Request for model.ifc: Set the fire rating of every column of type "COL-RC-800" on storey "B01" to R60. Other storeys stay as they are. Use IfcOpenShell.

First a look at what the model holds.

```python
import ifcopenshell
import ifcopenshell.util.element

model = ifcopenshell.open("model.ifc")
print(model.schema)
storey = next(s for s in model.by_type("IfcBuildingStorey") if s.Name == "B01")
columns = [e for e in ifcopenshell.util.element.get_decomposition(storey) if e.is_a("IfcColumn")]
seen = {}
for e in columns:
    element_type = ifcopenshell.util.element.get_type(e)
    key = (element_type.Name if element_type != e and element_type else None, ifcopenshell.util.element.get_pset(e, "Pset_ColumnCommon", "FireRating"))
    seen[key] = seen.get(key, 0) + 1
for (name, value), count in sorted(seen.items(), key=str):
    print(count, "x", name, "|", value)
```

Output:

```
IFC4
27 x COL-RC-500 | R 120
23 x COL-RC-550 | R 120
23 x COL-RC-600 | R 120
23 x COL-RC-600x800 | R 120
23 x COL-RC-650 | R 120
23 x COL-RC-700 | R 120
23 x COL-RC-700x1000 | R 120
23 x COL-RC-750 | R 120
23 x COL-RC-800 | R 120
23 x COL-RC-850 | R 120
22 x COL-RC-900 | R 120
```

```python
import ifcopenshell
import ifcopenshell.api.pset
import ifcopenshell.util.element

model = ifcopenshell.open("model.ifc")

storey = next(s for s in model.by_type("IfcBuildingStorey") if s.Name == "B01")
columns = [e for e in ifcopenshell.util.element.get_decomposition(storey) if e.is_a("IfcColumn")]

count = 0
for e in columns:
    element_type = ifcopenshell.util.element.get_type(e)
    if element_type in (None, e) or element_type.Name != "COL-RC-800":
        continue
    # add_pset returns the element's existing set when there is one.
    pset = ifcopenshell.api.pset.add_pset(model, product=e, name="Pset_ColumnCommon")
    ifcopenshell.api.pset.edit_pset(model, pset=pset, properties={"FireRating": "R60"})
    count += 1

print(count, "columns updated")

model.write("model_rev.ifc")
```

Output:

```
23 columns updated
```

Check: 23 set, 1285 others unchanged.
